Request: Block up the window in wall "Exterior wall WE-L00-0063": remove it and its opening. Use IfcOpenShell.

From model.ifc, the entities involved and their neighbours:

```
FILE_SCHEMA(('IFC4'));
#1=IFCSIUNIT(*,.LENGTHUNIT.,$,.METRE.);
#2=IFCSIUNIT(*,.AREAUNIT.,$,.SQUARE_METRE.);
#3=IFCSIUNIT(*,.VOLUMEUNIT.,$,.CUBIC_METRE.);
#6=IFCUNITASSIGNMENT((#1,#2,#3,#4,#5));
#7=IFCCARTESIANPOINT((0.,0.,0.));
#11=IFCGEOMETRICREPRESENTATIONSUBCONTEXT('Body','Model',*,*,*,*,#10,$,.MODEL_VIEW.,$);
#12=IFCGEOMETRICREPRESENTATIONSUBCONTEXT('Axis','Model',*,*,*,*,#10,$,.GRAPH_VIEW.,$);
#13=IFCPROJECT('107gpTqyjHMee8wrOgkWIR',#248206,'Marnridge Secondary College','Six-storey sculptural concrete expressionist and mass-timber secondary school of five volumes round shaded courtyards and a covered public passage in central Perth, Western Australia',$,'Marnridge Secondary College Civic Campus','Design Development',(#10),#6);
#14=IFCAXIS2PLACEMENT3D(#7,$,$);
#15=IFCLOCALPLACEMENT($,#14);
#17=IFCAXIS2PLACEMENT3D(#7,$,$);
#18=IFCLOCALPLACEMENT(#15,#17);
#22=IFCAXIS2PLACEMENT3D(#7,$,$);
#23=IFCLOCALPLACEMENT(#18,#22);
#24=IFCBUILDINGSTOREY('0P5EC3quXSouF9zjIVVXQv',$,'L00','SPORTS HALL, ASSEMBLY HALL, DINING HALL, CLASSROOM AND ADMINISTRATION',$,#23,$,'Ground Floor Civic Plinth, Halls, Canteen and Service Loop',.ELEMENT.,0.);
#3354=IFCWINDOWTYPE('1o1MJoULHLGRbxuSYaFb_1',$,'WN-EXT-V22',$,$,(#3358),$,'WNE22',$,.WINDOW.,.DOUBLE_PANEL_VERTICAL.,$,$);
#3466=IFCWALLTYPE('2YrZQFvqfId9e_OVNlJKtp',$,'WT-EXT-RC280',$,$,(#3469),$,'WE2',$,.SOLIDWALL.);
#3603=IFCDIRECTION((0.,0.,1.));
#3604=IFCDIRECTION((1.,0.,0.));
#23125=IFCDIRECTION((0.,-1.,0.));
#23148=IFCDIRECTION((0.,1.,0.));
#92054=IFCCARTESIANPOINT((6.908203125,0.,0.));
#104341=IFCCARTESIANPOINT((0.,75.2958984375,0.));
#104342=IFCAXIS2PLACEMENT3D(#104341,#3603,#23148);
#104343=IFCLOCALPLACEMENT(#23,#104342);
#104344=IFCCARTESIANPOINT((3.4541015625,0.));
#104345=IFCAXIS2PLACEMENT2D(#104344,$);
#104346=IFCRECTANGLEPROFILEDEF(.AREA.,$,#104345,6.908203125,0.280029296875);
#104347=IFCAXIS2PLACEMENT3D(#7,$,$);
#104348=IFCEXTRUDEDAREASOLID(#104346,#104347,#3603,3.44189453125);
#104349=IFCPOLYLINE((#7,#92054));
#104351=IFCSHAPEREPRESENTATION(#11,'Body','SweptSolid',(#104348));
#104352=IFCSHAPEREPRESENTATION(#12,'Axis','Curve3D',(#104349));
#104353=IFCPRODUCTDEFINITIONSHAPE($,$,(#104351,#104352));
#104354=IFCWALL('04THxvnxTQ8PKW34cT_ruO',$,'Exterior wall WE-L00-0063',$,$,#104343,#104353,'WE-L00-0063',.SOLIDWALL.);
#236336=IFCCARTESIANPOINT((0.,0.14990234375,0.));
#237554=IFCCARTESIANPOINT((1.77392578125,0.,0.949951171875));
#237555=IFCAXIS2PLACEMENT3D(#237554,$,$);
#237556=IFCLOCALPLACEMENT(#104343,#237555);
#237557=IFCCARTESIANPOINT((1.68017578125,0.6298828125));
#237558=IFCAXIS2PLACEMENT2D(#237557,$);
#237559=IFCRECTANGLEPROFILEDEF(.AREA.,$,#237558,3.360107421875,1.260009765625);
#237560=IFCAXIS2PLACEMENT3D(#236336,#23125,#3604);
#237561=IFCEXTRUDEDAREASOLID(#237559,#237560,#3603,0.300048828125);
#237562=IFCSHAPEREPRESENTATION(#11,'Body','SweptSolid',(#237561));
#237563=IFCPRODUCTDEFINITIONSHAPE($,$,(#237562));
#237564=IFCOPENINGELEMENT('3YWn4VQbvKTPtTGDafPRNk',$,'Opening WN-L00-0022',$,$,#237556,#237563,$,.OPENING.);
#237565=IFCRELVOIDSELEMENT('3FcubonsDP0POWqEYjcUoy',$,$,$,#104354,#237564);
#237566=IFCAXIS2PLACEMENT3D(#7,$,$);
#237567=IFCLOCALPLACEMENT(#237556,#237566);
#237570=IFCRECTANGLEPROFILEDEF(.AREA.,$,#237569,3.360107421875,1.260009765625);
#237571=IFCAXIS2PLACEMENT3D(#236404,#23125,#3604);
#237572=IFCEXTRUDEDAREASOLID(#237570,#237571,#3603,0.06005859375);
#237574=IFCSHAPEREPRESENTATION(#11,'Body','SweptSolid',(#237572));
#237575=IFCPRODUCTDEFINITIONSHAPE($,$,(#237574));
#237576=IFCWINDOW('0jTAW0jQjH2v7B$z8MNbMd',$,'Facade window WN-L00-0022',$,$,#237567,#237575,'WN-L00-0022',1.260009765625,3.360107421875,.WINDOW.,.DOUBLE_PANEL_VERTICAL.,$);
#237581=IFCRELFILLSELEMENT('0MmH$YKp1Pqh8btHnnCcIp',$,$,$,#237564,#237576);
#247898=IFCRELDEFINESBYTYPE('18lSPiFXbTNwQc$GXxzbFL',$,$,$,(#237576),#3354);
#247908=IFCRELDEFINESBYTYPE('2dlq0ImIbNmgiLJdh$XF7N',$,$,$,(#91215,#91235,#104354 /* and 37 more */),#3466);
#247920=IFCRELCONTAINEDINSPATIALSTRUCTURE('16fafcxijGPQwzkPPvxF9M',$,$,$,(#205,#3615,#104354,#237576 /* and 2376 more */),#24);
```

```python
import ifcopenshell
import ifcopenshell.api.feature
import ifcopenshell.api.root
import ifcopenshell.geom
import ifcopenshell.util.shape

model = ifcopenshell.open("model.ifc")
settings = ifcopenshell.geom.settings()


def volume(element):
    """Net volume in cubic metres, openings subtracted."""
    shape = ifcopenshell.geom.create_shape(settings, element)
    return ifcopenshell.util.shape.get_volume(shape.geometry)


window = model.by_guid("0jTAW0jQjH2v7B$z8MNbMd")
opening = window.FillsVoids[0].RelatingOpeningElement
wall = opening.VoidsElements[0].RelatingBuildingElement
before = volume(wall)

ifcopenshell.api.root.remove_product(model, product=window)
ifcopenshell.api.feature.remove_feature(model, feature=opening)

after = volume(wall)

print(f"wall volume {before:.3f} -> {after:.3f} m3")

model.write("model_rev.ifc")
```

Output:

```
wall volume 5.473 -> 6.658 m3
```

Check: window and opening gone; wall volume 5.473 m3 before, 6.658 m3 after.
